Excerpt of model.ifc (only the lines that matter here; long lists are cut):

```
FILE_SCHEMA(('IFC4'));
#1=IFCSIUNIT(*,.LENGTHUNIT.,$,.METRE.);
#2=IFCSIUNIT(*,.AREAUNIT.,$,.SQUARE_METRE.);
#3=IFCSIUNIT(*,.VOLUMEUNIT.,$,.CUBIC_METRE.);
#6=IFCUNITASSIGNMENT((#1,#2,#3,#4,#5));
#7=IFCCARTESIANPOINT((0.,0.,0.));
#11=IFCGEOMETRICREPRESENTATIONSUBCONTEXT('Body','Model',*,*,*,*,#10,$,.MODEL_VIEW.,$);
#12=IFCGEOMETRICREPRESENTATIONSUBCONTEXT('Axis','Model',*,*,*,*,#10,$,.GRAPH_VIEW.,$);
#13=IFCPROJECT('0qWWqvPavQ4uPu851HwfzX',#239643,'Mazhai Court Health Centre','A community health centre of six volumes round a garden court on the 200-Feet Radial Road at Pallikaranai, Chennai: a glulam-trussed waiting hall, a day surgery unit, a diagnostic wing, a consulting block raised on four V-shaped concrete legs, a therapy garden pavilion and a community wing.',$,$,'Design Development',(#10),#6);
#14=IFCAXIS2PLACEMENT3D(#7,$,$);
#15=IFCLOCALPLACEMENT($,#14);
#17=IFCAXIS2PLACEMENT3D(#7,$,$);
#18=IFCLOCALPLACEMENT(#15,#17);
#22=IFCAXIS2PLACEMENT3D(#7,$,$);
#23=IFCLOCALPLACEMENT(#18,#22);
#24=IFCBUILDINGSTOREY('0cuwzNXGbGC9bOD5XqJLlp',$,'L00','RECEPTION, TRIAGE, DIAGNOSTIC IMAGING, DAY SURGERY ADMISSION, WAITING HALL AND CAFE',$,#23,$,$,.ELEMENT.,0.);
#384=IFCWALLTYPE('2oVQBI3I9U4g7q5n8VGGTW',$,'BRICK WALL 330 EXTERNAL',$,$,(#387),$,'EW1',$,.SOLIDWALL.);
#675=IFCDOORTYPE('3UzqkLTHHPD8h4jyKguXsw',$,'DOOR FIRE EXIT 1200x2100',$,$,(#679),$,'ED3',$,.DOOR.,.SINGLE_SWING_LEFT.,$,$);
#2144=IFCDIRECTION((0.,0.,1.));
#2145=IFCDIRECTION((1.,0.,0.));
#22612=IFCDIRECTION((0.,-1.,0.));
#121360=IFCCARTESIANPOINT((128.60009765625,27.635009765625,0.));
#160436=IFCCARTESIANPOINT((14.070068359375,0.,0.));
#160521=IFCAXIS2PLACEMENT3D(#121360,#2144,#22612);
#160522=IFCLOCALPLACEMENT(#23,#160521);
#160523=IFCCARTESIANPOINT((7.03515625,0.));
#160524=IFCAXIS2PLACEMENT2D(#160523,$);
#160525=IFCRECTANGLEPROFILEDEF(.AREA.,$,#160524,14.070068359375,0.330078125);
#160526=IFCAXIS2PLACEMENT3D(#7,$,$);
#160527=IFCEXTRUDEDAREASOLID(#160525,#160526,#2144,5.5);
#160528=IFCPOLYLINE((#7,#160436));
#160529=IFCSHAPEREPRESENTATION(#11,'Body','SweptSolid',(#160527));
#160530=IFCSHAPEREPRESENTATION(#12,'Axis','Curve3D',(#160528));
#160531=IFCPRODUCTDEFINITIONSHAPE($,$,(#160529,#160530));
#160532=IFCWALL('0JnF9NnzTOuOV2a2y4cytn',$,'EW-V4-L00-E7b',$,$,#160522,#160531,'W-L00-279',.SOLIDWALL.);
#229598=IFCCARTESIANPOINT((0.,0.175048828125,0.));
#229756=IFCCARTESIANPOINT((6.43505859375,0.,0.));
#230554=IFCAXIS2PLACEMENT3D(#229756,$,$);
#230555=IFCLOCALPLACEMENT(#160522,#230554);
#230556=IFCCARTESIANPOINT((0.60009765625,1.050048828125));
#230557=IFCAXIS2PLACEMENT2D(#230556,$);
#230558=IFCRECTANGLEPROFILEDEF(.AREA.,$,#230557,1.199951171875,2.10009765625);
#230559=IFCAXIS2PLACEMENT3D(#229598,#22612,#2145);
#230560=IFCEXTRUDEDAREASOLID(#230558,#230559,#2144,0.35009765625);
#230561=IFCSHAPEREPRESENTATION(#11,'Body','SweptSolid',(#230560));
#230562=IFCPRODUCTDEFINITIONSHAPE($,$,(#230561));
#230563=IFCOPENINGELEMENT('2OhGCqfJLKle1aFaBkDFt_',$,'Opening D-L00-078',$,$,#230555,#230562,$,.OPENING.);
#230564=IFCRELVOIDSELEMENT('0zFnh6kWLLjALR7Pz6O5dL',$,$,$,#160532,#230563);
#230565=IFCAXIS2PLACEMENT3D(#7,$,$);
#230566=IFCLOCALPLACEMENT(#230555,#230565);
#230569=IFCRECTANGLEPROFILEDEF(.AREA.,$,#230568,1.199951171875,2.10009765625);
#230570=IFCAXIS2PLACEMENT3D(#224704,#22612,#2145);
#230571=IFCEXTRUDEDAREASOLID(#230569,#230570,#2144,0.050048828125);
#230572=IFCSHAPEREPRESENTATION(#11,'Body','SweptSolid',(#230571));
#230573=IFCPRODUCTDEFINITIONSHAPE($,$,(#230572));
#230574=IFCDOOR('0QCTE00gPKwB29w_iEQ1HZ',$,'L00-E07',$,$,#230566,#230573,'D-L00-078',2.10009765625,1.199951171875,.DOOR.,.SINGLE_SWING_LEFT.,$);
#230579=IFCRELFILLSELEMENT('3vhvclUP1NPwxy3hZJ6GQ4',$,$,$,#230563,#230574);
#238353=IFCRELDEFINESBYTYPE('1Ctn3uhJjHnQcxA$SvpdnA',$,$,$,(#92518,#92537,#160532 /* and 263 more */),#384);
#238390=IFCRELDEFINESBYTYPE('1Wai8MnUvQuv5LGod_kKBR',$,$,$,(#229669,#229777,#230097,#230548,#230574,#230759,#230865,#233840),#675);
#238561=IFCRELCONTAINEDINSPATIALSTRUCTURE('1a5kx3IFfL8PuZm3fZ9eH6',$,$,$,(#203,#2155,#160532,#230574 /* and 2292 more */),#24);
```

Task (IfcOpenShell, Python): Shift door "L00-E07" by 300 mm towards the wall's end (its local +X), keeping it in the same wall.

```python
import ifcopenshell
import ifcopenshell.api.geometry
import ifcopenshell.util.placement

model = ifcopenshell.open("model.ifc")

door = model.by_guid("0QCTE00gPKwB29w_iEQ1HZ")
opening = door.FillsVoids[0].RelatingOpeningElement
wall = opening.VoidsElements[0].RelatingBuildingElement

wall_matrix = ifcopenshell.util.placement.get_local_placement(wall.ObjectPlacement)
shift = wall_matrix[:3, 0] * 0.3
before = ifcopenshell.util.placement.get_local_placement(door.ObjectPlacement)[:3, 3].copy()

# The door is placed relative to its opening, so it follows when the opening moves.
matrix = ifcopenshell.util.placement.get_local_placement(opening.ObjectPlacement)
matrix[:3, 3] += shift
ifcopenshell.api.geometry.edit_object_placement(
    model, product=opening, matrix=matrix, is_si=False, should_transform_children=True
)

after = ifcopenshell.util.placement.get_local_placement(door.ObjectPlacement)[:3, 3]
print("door moved by", (after - before).round(3) + 0.0)

model.write("model_updated.ifc")
```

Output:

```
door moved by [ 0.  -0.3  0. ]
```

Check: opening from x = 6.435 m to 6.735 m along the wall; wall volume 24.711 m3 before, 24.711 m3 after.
